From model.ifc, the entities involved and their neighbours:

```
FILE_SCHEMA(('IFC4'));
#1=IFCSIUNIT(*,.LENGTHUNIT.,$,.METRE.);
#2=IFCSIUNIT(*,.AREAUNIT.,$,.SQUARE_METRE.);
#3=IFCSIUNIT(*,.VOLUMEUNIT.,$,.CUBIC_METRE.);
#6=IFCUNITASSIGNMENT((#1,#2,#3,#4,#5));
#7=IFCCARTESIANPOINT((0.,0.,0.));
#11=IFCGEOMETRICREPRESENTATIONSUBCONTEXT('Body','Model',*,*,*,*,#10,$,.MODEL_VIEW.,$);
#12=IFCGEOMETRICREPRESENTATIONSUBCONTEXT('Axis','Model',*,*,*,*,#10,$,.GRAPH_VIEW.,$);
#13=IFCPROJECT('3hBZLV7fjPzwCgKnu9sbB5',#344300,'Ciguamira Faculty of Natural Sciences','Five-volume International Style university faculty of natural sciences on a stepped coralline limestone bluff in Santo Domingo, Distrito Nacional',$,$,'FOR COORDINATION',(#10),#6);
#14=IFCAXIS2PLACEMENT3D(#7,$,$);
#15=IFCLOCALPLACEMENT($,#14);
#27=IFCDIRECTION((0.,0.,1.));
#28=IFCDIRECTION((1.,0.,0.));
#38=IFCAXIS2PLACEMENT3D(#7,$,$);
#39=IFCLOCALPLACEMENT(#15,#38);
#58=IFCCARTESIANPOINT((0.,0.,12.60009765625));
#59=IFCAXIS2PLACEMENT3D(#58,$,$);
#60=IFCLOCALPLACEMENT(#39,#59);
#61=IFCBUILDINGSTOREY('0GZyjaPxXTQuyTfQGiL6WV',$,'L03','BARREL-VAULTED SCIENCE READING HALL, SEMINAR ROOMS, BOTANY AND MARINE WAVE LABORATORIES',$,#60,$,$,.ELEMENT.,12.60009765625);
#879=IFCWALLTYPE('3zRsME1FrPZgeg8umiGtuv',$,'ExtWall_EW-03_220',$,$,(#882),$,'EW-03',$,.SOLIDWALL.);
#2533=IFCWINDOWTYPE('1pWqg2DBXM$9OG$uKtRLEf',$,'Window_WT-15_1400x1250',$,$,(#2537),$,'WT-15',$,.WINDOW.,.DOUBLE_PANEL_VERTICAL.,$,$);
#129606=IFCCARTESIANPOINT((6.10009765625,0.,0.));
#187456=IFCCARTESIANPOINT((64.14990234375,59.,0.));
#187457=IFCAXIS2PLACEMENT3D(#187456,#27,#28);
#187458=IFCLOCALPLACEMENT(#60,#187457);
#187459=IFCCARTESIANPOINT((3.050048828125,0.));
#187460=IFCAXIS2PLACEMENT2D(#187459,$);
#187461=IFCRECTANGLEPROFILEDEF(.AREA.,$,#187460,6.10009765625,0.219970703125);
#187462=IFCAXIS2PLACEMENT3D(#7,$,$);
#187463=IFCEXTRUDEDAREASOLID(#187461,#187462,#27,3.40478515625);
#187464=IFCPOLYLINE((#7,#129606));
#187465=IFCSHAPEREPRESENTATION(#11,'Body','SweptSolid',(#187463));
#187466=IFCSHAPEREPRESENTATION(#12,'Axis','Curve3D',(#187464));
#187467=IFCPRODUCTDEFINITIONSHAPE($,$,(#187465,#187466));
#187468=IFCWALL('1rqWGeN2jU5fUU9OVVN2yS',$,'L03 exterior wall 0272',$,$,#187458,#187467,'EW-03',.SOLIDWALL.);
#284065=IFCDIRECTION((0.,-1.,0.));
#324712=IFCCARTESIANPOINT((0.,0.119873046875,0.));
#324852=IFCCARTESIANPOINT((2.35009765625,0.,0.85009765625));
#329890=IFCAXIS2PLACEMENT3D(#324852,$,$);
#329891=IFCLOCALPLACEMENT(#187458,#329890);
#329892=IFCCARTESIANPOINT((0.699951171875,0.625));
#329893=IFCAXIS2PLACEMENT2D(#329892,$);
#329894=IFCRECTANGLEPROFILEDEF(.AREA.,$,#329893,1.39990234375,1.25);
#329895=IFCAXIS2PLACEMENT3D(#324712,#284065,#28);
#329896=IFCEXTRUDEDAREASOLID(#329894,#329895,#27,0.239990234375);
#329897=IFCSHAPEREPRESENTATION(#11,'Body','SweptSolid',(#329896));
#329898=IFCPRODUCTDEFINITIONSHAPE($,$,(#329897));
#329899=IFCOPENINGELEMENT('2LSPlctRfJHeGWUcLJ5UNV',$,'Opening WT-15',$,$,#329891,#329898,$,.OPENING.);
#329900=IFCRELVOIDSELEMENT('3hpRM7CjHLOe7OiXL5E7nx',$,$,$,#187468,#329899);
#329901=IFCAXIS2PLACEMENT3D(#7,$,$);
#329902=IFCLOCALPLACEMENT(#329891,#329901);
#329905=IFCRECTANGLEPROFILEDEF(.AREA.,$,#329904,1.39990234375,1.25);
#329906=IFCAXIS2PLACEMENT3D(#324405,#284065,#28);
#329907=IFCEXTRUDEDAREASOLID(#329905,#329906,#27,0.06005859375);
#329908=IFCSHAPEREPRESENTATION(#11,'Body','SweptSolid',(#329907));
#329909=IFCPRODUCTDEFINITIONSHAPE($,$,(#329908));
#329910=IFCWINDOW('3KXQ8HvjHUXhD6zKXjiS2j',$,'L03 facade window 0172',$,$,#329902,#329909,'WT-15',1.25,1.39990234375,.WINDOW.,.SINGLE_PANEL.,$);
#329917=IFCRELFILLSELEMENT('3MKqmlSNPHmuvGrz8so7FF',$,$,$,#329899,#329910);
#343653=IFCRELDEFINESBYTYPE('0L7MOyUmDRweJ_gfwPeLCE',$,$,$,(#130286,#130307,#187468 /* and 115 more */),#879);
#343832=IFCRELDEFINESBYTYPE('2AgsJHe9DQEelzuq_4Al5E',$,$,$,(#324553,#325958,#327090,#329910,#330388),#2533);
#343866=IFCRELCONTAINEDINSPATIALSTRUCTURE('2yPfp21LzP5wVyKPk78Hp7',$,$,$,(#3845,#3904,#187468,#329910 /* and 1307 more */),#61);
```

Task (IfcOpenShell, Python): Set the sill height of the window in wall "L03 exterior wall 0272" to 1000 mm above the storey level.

```python
import numpy as np
import ifcopenshell
import ifcopenshell.api.geometry
import ifcopenshell.geom
import ifcopenshell.util.element
import ifcopenshell.util.placement
import ifcopenshell.util.shape
import ifcopenshell.util.unit

model = ifcopenshell.open("model.ifc")
unit_scale = ifcopenshell.util.unit.calculate_unit_scale(model)

window = model.by_guid("3KXQ8HvjHUXhD6zKXjiS2j")
opening = window.FillsVoids[0].RelatingOpeningElement
storey = ifcopenshell.util.element.get_container(window, ifc_class="IfcBuildingStorey")
level = ifcopenshell.util.placement.get_local_placement(storey.ObjectPlacement)[2, 3]

# The opening's origin need not be at the sill, so measure its lowest point.
shape = ifcopenshell.geom.create_shape(ifcopenshell.geom.settings(), opening)
bottom = ifcopenshell.util.shape.get_shape_bottom_elevation(shape, shape.geometry) / unit_scale
dz = level + 1.0 - bottom

shift = np.array([0.0, 0.0, dz])
# The window is placed relative to its opening, so it follows when the opening moves.
matrix = ifcopenshell.util.placement.get_local_placement(opening.ObjectPlacement)
matrix[:3, 3] += shift
ifcopenshell.api.geometry.edit_object_placement(
    model, product=opening, matrix=matrix, is_si=False, should_transform_children=True
)

print(f"moved by {dz * unit_scale:+.3f} m")

model.write("model_v2.ifc")
```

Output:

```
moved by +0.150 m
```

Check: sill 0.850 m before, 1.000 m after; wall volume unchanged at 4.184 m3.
